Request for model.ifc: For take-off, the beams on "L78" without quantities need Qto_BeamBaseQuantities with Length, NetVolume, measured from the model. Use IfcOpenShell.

First a look at what the model holds.

```python
import ifcopenshell
import ifcopenshell.util.element
import ifcopenshell.util.unit

model = ifcopenshell.open("model.ifc")
print(model.schema)
for unit_type in ("LENGTHUNIT", "AREAUNIT", "VOLUMEUNIT"):
    print(unit_type, ifcopenshell.util.unit.calculate_unit_scale(model, unit_type))
storey = next(s for s in model.by_type("IfcBuildingStorey") if s.Name == "L78")
beams = [e for e in ifcopenshell.util.element.get_decomposition(storey) if e.is_a("IfcBeam")]
for e in sorted(beams, key=lambda e: e.id()):
    print(e.id(), e.is_a(), e.Name, list(ifcopenshell.util.element.get_psets(e, qtos_only=True)), sep=" | ")
```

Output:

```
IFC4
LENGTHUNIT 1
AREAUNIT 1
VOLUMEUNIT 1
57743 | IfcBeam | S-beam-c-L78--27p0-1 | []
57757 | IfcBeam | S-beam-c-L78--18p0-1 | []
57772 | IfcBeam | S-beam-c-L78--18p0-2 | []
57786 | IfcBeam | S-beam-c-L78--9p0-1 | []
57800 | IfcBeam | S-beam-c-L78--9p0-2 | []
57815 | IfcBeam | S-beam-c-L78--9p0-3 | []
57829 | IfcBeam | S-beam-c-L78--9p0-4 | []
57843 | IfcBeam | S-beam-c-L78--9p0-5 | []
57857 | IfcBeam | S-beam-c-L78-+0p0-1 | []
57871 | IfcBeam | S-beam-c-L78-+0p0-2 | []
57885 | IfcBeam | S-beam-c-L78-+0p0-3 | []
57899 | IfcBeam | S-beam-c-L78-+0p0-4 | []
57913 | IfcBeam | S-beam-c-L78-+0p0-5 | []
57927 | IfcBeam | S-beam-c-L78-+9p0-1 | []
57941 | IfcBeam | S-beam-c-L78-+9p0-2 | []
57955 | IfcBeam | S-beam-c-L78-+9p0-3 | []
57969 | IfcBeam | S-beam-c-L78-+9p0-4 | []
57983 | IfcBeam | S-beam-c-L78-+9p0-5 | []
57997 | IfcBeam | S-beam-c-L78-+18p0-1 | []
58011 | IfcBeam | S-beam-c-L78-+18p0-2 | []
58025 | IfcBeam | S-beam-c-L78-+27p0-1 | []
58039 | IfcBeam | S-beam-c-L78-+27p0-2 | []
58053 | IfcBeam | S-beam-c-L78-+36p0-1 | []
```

```python
import ifcopenshell
import ifcopenshell.api.pset
import ifcopenshell.geom
import ifcopenshell.util.element
import ifcopenshell.util.shape
import ifcopenshell.util.unit

model = ifcopenshell.open("model.ifc")
unit_scale = ifcopenshell.util.unit.calculate_unit_scale(model)
volume_scale = ifcopenshell.util.unit.calculate_unit_scale(model, "VOLUMEUNIT")
settings = ifcopenshell.geom.settings()

storey = next(s for s in model.by_type("IfcBuildingStorey") if s.Name == "L78")
beams = [e for e in ifcopenshell.util.element.get_decomposition(storey) if e.is_a("IfcBeam")]

for e in sorted(beams, key=lambda e: e.id()):
    if ifcopenshell.util.element.get_psets(e, qtos_only=True, should_inherit=False):
        continue
    # Geometry comes back in metres, in the element's own axes.
    shape = ifcopenshell.geom.create_shape(settings, e)
    values = {
        "Length": ifcopenshell.util.shape.get_max_xyz(shape.geometry) / unit_scale,
        "NetVolume": ifcopenshell.util.shape.get_volume(shape.geometry) / volume_scale,
    }
    qto = ifcopenshell.api.pset.add_qto(model, product=e, name="Qto_BeamBaseQuantities")
    ifcopenshell.api.pset.edit_qto(model, qto=qto, properties=values)
    print(e.id(), {k: round(v, 3) for k, v in values.items()})

model.write("model_edited.ifc")
```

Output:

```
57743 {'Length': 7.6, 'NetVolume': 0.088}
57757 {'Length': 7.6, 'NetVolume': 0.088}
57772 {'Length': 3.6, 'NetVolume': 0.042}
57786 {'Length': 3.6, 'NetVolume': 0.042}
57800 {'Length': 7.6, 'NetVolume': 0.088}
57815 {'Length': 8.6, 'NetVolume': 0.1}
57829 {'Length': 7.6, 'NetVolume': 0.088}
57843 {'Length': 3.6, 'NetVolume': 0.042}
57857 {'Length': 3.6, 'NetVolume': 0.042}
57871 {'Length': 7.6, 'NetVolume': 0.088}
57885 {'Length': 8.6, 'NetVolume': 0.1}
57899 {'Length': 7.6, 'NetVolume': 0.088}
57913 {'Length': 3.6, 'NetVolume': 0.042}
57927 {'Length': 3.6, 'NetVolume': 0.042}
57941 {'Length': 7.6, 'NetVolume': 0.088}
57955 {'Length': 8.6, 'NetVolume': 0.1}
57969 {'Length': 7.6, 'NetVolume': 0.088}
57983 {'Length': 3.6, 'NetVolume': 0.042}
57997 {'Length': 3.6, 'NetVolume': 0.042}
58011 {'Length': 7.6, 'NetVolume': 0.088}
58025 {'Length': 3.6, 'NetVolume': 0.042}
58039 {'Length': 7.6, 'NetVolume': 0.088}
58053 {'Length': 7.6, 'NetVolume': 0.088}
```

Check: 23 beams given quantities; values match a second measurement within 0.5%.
